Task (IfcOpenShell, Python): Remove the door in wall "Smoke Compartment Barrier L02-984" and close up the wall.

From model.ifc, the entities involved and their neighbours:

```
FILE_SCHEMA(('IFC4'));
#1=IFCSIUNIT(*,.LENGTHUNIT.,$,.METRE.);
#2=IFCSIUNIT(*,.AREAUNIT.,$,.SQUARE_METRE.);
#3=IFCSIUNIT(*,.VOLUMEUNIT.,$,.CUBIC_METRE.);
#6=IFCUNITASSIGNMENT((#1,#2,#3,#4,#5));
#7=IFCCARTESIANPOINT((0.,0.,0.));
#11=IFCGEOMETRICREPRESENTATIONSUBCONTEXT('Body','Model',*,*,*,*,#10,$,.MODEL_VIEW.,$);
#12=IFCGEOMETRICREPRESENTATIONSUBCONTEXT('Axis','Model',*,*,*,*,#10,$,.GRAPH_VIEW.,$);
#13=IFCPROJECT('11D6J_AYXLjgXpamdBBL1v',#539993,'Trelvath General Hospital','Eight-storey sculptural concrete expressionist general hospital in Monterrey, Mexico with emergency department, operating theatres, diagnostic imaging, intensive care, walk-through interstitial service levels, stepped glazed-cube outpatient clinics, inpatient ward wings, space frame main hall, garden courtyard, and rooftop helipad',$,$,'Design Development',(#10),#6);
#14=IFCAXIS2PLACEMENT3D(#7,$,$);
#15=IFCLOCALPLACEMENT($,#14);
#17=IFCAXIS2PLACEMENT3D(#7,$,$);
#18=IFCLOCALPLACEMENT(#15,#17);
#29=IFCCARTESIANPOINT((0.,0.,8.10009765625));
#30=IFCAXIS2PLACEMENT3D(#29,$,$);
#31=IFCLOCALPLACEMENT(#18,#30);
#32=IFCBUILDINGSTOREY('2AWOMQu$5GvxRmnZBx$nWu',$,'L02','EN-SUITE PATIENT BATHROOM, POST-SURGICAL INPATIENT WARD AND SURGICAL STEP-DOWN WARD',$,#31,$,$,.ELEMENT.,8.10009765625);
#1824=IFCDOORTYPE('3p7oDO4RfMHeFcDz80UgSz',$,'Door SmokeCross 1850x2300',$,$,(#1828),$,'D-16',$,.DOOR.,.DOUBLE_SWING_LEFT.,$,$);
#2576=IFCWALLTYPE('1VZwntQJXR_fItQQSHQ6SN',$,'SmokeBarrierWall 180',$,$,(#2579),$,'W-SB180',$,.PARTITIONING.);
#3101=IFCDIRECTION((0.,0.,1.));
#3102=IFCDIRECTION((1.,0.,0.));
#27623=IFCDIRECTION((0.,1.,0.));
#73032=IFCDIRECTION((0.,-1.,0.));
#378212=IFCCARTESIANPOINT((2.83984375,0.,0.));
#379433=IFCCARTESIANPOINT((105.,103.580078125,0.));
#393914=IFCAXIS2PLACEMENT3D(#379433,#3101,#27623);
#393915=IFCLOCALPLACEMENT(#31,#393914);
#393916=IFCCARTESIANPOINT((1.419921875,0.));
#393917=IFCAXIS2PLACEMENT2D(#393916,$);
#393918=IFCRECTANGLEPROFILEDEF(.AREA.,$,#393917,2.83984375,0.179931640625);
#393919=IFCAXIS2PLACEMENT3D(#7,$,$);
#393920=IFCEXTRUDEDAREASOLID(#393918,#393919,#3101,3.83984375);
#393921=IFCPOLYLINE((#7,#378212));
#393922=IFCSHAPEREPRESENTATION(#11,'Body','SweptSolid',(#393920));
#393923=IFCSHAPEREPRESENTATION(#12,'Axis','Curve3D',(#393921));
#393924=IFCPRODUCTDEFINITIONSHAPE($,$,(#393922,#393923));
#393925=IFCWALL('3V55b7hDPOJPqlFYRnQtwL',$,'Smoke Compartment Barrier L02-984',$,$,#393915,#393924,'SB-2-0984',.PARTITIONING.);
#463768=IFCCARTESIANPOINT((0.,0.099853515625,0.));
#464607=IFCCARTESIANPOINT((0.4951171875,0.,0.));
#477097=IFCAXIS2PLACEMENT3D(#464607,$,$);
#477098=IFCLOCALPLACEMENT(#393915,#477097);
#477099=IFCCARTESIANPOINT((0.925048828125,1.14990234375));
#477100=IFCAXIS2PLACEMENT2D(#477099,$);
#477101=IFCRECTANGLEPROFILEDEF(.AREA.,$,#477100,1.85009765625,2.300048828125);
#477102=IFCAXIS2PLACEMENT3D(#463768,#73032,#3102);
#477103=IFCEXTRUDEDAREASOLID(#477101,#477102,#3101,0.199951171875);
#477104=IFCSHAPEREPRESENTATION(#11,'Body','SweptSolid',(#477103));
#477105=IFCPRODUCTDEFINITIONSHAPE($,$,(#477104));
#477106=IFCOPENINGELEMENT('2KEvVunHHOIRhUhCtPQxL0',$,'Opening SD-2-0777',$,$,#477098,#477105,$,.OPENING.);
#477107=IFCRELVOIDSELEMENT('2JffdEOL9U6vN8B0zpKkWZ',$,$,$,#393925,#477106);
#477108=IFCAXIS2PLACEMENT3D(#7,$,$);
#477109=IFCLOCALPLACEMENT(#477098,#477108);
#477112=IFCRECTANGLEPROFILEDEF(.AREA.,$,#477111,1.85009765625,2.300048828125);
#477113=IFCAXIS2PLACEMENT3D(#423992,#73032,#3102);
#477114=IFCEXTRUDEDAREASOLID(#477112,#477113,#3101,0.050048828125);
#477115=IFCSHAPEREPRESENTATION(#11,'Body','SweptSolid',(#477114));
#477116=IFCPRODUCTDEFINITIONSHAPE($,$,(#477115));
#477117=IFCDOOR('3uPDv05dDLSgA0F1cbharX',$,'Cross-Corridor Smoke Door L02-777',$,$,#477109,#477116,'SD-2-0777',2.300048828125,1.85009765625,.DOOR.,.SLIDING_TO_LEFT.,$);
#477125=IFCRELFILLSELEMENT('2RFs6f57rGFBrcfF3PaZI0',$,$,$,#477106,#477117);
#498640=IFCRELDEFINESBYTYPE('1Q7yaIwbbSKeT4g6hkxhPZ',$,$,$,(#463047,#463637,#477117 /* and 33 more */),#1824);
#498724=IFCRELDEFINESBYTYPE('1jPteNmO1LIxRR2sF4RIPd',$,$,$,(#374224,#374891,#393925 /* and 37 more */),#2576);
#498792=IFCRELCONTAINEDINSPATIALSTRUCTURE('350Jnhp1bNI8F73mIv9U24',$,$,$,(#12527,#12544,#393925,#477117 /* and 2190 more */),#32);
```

```python
import ifcopenshell
import ifcopenshell.api.feature
import ifcopenshell.api.root
import ifcopenshell.geom
import ifcopenshell.util.shape

model = ifcopenshell.open("model.ifc")
settings = ifcopenshell.geom.settings()


def volume(element):
    """Net volume in cubic metres, openings subtracted."""
    shape = ifcopenshell.geom.create_shape(settings, element)
    return ifcopenshell.util.shape.get_volume(shape.geometry)


door = model.by_id(477117)
opening = door.FillsVoids[0].RelatingOpeningElement
wall = opening.VoidsElements[0].RelatingBuildingElement
before = volume(wall)

ifcopenshell.api.root.remove_product(model, product=door)
ifcopenshell.api.feature.remove_feature(model, feature=opening)

after = volume(wall)

print(f"wall volume {before:.3f} -> {after:.3f} m3")

model.write("model_rev.ifc")
```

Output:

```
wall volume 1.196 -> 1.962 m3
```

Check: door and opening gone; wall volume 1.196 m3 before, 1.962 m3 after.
